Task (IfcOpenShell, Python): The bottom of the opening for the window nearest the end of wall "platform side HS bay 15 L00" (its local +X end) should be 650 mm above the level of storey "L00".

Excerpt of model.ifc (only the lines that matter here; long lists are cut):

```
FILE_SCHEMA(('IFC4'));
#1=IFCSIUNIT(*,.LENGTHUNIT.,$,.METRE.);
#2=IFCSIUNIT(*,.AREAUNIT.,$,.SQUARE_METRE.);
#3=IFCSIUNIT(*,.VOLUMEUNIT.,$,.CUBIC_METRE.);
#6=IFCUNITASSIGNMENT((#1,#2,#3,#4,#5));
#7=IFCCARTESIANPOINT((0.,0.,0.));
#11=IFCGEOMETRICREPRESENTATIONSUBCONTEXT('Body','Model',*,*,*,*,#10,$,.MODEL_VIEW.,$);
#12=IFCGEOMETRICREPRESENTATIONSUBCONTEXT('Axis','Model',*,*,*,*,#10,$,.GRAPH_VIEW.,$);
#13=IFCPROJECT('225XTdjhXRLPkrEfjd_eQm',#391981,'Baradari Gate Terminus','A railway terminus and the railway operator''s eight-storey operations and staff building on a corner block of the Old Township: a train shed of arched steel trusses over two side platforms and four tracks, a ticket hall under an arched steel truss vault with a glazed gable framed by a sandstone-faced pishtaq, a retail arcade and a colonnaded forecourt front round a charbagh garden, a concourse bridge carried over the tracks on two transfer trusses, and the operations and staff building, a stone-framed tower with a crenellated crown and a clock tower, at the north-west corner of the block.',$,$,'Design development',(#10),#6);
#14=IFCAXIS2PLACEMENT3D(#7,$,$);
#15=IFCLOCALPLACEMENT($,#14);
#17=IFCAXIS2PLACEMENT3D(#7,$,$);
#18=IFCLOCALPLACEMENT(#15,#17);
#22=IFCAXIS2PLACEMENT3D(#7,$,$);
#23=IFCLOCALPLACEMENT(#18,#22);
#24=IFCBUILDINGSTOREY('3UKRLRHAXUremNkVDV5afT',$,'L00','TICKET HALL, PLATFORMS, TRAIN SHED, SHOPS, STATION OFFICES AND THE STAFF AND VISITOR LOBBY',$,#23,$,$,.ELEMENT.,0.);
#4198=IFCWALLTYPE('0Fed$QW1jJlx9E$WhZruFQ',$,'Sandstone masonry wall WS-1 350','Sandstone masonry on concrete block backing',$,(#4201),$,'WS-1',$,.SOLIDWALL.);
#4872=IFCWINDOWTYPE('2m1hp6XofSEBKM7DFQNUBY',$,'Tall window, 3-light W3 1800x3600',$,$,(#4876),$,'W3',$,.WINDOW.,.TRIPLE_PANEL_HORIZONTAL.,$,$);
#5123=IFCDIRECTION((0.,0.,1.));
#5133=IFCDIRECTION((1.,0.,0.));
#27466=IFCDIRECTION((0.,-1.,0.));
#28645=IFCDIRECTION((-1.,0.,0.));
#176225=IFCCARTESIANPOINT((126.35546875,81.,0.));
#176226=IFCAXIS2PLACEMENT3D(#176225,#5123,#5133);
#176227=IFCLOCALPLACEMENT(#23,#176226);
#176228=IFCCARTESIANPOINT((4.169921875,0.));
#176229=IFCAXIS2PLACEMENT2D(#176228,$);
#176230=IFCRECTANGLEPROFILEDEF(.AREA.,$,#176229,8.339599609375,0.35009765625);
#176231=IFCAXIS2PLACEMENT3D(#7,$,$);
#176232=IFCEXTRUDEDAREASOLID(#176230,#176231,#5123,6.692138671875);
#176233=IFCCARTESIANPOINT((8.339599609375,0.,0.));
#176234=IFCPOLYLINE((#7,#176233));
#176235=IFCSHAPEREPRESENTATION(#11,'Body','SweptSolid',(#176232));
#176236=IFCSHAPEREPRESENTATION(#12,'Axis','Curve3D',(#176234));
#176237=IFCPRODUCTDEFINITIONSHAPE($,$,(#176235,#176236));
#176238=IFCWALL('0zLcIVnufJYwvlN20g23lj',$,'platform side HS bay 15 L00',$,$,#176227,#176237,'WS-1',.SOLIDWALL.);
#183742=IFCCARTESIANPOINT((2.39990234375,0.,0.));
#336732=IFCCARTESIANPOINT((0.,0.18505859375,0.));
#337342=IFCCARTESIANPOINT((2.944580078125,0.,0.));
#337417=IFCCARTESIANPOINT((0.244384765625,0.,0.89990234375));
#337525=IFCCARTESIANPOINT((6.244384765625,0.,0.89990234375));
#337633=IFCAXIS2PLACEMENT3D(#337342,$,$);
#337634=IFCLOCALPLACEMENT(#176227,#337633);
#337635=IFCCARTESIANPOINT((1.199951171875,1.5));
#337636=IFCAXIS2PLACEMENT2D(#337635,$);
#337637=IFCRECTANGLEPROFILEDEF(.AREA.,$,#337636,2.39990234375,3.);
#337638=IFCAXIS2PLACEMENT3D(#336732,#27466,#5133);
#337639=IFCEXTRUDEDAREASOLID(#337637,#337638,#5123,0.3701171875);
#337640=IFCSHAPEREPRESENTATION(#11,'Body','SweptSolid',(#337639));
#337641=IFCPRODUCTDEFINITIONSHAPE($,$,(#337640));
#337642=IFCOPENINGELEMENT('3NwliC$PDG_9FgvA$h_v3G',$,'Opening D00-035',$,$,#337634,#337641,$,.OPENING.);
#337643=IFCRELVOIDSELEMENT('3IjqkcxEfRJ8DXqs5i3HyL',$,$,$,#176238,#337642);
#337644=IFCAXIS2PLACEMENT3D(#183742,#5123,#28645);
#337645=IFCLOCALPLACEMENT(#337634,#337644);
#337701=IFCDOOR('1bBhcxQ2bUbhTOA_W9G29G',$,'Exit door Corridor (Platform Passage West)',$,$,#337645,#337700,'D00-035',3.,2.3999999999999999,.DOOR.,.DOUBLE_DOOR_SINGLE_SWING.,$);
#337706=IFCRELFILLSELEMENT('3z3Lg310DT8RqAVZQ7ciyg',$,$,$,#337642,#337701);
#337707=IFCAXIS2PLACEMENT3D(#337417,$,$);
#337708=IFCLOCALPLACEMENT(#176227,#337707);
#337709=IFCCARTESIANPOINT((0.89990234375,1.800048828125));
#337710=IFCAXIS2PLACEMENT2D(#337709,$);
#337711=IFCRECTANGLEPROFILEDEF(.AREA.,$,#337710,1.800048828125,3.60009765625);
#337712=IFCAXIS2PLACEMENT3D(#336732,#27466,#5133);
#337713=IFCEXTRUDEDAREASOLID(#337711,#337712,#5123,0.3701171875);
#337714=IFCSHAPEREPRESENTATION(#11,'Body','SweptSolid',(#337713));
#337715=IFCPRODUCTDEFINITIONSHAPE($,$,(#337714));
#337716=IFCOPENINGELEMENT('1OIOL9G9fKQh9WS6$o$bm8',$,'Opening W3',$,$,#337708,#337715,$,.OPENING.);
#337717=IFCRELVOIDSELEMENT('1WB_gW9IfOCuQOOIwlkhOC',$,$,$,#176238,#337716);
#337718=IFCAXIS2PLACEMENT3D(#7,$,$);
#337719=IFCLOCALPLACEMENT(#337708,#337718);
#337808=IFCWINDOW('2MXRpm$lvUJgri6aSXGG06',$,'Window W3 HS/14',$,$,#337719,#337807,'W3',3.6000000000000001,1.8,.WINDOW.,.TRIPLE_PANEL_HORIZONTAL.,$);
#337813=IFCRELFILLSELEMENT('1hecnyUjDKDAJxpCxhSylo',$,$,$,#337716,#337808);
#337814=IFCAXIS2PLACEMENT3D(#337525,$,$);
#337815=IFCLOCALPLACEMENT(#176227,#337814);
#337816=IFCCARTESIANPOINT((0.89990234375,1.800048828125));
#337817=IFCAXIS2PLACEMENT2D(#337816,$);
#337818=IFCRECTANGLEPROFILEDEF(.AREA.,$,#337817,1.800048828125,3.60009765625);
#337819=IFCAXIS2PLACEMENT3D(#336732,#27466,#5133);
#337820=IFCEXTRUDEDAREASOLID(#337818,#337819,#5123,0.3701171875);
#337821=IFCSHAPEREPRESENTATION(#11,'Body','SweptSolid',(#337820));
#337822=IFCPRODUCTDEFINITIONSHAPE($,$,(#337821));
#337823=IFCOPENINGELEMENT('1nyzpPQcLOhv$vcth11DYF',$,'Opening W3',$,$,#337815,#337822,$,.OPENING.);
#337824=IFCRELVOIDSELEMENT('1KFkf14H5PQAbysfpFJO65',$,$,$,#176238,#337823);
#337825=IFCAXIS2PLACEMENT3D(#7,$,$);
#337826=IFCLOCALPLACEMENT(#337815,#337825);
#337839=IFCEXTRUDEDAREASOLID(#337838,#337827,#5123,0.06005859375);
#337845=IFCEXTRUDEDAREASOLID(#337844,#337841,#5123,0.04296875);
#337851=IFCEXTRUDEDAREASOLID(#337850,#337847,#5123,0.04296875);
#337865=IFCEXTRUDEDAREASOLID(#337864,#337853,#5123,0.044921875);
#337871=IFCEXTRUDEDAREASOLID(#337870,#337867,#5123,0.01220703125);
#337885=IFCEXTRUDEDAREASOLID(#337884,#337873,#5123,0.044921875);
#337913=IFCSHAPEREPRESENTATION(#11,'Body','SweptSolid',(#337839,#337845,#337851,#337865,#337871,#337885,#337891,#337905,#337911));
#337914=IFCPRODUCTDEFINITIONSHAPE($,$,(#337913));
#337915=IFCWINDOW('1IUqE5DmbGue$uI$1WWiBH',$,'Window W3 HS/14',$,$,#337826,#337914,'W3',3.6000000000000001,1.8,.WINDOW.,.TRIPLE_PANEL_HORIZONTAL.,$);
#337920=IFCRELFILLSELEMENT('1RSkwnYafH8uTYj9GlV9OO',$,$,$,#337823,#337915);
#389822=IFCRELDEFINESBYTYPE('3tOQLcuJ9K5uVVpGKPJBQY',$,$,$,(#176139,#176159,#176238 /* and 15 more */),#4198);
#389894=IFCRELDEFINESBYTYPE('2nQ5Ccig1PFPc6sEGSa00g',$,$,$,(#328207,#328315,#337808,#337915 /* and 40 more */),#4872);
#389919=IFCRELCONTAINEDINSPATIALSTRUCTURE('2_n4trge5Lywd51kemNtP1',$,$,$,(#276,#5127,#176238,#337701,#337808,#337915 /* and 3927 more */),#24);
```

```python
import numpy as np
import ifcopenshell
import ifcopenshell.api.geometry
import ifcopenshell.geom
import ifcopenshell.util.element
import ifcopenshell.util.placement
import ifcopenshell.util.shape
import ifcopenshell.util.unit

model = ifcopenshell.open("model.ifc")
unit_scale = ifcopenshell.util.unit.calculate_unit_scale(model)

window = model.by_id(337915)
opening = window.FillsVoids[0].RelatingOpeningElement
storey = ifcopenshell.util.element.get_container(window, ifc_class="IfcBuildingStorey")
level = ifcopenshell.util.placement.get_local_placement(storey.ObjectPlacement)[2, 3]

# The opening's origin need not be at the sill, so measure its lowest point.
shape = ifcopenshell.geom.create_shape(ifcopenshell.geom.settings(), opening)
bottom = ifcopenshell.util.shape.get_shape_bottom_elevation(shape, shape.geometry) / unit_scale
dz = level + 0.65 - bottom

shift = np.array([0.0, 0.0, dz])
# The window is placed relative to its opening, so it follows when the opening moves.
matrix = ifcopenshell.util.placement.get_local_placement(opening.ObjectPlacement)
matrix[:3, 3] += shift
ifcopenshell.api.geometry.edit_object_placement(
    model, product=opening, matrix=matrix, is_si=False, should_transform_children=True
)

print(f"moved by {dz * unit_scale:+.3f} m")

model.write("model_v2.ifc")
```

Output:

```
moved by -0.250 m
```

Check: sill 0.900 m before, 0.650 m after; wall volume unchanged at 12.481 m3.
